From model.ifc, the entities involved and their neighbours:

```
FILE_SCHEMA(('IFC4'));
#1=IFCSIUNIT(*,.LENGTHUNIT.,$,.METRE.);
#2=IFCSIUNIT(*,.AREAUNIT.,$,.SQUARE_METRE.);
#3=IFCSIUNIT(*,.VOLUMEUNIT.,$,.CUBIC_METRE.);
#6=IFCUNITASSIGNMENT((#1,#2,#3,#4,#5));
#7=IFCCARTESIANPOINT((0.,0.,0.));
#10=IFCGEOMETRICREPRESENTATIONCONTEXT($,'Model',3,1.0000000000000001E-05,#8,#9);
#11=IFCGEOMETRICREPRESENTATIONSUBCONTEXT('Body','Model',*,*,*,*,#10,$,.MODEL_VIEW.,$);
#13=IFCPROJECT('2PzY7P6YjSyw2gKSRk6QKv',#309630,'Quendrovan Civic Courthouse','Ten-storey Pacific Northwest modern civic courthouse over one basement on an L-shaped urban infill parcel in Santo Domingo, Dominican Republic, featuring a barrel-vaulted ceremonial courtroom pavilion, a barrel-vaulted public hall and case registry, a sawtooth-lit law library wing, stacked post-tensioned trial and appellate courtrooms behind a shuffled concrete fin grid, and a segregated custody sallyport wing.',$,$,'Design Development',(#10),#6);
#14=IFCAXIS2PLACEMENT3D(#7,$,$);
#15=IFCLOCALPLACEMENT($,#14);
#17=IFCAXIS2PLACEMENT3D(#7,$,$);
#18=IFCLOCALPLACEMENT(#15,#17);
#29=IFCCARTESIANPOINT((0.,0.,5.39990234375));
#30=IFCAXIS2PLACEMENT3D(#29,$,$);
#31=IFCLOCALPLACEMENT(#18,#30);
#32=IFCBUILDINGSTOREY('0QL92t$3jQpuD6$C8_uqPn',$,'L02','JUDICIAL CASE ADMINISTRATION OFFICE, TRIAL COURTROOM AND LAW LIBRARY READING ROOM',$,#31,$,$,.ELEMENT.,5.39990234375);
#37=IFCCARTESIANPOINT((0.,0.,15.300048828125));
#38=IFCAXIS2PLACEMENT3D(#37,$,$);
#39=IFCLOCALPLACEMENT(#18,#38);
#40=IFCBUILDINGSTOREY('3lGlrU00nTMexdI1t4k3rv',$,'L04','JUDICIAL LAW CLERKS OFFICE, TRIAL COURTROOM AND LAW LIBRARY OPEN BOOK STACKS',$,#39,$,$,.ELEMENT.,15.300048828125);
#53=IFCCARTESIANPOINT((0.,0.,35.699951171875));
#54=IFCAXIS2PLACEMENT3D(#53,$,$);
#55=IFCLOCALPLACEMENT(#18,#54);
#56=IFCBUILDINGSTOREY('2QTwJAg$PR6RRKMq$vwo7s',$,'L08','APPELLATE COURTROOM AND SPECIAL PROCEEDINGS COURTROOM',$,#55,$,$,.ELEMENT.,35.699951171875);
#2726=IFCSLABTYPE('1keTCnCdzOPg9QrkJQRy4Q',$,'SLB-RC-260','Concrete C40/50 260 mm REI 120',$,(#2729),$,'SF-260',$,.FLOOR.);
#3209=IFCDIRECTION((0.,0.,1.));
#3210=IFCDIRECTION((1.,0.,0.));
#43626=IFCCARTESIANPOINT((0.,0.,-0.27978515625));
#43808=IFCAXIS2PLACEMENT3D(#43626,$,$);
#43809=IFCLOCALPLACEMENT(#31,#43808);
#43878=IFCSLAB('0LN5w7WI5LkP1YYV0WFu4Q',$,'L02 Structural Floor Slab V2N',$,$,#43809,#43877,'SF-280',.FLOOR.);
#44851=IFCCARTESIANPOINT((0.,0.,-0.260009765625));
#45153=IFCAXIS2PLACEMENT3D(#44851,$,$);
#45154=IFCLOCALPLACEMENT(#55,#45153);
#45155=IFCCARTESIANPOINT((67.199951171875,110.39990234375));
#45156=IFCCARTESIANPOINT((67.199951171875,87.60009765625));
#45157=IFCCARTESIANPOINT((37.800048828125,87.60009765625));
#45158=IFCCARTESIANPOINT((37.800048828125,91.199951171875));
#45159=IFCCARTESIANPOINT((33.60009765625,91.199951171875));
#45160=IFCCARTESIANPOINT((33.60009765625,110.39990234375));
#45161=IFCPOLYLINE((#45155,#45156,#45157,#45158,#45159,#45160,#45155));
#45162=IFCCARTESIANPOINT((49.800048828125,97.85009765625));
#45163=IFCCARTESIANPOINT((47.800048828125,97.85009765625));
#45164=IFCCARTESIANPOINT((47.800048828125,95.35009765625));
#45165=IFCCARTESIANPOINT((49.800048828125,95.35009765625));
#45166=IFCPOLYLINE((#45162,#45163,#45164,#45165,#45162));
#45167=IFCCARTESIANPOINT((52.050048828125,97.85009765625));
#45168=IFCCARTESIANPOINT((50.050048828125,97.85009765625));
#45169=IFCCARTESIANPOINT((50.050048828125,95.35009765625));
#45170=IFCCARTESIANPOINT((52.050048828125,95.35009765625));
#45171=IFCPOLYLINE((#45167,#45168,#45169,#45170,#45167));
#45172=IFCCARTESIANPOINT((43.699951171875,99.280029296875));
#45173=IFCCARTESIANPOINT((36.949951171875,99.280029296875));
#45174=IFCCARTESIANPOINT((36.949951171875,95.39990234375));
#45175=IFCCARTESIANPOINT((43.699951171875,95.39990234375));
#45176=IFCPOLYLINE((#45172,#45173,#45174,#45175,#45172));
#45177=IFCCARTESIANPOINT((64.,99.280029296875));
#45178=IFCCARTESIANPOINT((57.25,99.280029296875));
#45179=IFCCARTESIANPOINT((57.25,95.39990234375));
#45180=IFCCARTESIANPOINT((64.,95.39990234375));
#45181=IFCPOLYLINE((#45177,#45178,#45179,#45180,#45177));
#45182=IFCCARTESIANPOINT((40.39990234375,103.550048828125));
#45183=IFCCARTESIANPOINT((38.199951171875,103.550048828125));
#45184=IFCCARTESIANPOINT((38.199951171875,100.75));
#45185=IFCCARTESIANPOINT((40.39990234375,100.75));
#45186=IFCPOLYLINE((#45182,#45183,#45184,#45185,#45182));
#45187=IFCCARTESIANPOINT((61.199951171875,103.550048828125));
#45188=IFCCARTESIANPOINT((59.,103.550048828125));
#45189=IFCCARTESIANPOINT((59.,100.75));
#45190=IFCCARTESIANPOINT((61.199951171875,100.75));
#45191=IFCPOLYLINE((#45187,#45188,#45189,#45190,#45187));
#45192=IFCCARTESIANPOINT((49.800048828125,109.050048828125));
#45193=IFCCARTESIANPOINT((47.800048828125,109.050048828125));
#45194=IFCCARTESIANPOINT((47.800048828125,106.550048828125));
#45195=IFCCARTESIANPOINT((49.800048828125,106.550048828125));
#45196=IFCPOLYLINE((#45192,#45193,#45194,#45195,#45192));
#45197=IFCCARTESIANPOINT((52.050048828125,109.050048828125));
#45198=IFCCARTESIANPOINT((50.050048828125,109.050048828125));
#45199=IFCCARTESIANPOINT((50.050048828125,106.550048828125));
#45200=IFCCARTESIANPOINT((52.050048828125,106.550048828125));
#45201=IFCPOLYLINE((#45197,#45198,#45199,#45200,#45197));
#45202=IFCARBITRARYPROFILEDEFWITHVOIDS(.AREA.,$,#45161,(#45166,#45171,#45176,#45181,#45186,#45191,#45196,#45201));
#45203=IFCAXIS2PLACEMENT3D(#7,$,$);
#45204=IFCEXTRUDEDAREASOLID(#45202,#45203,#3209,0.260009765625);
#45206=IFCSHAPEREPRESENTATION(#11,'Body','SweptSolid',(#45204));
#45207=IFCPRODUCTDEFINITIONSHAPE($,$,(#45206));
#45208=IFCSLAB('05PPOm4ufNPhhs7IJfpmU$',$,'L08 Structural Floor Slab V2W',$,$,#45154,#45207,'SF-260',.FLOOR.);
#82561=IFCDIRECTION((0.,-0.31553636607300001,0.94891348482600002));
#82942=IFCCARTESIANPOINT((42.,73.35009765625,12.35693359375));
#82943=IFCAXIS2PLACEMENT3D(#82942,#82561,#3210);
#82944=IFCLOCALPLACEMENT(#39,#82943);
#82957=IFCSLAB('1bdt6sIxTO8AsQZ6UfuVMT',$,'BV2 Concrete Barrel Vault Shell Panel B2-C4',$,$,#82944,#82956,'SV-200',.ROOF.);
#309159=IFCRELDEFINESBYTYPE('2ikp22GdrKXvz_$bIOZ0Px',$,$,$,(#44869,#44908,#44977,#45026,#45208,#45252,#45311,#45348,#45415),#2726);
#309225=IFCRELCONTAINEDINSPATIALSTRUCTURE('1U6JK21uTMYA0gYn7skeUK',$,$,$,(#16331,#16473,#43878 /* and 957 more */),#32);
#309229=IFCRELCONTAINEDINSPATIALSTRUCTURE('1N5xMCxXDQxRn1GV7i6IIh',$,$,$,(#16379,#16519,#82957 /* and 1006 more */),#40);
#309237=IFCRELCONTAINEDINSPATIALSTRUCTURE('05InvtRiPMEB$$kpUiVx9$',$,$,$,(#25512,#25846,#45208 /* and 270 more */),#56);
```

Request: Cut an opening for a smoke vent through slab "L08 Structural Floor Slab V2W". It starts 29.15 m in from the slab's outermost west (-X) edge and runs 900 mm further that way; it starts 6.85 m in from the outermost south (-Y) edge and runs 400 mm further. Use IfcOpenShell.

```python
import numpy as np
import ifcopenshell
import ifcopenshell.api.feature
import ifcopenshell.api.geometry
import ifcopenshell.api.root
import ifcopenshell.geom
import ifcopenshell.util.placement
import ifcopenshell.util.representation
import ifcopenshell.util.shape
import ifcopenshell.util.unit

model = ifcopenshell.open("model.ifc")
unit_scale = ifcopenshell.util.unit.calculate_unit_scale(model)
settings = ifcopenshell.geom.settings()


def volume(element):
    """Net volume in cubic metres, openings subtracted."""
    shape = ifcopenshell.geom.create_shape(settings, element)
    return ifcopenshell.util.shape.get_volume(shape.geometry)


slab = model.by_guid("05PPOm4ufNPhhs7IJfpmU$")
before = volume(slab)

# Extent in the slab's own axes, in metres. The edges named are its -X and -Y sides.
slab_shape = ifcopenshell.geom.create_shape(settings, slab)
vertices = ifcopenshell.util.shape.get_vertices(slab_shape.geometry)
x_min, y_min, bottom = vertices.min(axis=0)
top = vertices[:, 2].max()

opening = ifcopenshell.api.root.create_entity(model, ifc_class="IfcOpeningElement", name="Smoke vent opening", predefined_type="OPENING")
context = ifcopenshell.util.representation.get_context(model, "Model", "Body", "MODEL_VIEW")
width, depth = 0.9, 0.4
outline = [(0.0, 0.0), (width, 0.0), (width, depth), (0.0, depth), (0.0, 0.0)]
# Overshoot both faces by 50 mm so the cut is clean.
shape = ifcopenshell.api.geometry.add_slab_representation(
    model, context=context, depth=top - bottom + 0.1, polyline=outline
)
ifcopenshell.api.geometry.assign_representation(model, product=opening, representation=shape)

matrix = ifcopenshell.util.placement.get_local_placement(slab.ObjectPlacement)
matrix[:, 3] = matrix @ np.append(np.array([x_min + 29.15, y_min + 6.85, bottom - 0.05]) / unit_scale, 1.0)
ifcopenshell.api.geometry.edit_object_placement(model, product=opening, matrix=matrix, is_si=False)
ifcopenshell.api.feature.add_feature(model, feature=opening, element=slab)

after = volume(slab)

print(f"slab volume {before:.3f} -> {after:.3f} m3")

model.write("model_updated.ifc")
```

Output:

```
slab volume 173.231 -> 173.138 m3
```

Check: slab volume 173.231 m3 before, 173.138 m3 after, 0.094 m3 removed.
